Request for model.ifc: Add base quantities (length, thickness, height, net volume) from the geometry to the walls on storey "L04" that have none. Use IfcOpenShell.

First a look at what the model holds.

```python
import ifcopenshell
import ifcopenshell.util.element
import ifcopenshell.util.unit

model = ifcopenshell.open("model.ifc")
print(model.schema)
for unit_type in ("LENGTHUNIT", "AREAUNIT", "VOLUMEUNIT"):
    print(unit_type, ifcopenshell.util.unit.calculate_unit_scale(model, unit_type))
storey = next(s for s in model.by_type("IfcBuildingStorey") if s.Name == "L04")
walls = [e for e in ifcopenshell.util.element.get_decomposition(storey) if e.is_a("IfcWall")]
for e in sorted(walls, key=lambda e: e.id()):
    print(e.id(), e.is_a(), e.Name, list(ifcopenshell.util.element.get_psets(e, qtos_only=True)), sep=" | ")
```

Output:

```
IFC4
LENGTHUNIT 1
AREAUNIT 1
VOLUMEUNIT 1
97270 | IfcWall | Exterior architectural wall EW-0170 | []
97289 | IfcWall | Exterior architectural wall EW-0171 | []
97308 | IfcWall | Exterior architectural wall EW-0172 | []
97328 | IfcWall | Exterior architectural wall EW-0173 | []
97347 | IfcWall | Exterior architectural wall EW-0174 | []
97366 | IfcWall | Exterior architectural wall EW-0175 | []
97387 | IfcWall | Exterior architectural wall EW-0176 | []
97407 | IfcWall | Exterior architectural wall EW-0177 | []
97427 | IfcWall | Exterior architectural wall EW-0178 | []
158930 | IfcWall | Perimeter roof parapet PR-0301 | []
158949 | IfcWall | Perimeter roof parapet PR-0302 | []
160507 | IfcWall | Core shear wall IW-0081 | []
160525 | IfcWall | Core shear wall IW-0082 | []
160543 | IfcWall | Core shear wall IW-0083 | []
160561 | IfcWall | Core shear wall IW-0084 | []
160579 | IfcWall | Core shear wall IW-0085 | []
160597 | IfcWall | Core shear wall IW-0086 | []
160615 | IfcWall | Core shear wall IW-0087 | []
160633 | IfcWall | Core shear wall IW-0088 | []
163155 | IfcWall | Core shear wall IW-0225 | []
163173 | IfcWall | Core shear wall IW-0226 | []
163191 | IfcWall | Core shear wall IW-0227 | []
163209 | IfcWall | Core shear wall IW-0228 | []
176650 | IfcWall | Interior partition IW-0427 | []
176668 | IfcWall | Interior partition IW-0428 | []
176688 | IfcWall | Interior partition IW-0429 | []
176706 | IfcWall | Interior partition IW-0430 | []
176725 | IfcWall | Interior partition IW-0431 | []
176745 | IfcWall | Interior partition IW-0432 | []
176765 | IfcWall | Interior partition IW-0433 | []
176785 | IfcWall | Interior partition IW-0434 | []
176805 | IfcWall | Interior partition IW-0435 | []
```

```python
import ifcopenshell
import ifcopenshell.api.pset
import ifcopenshell.geom
import ifcopenshell.util.element
import ifcopenshell.util.shape
import ifcopenshell.util.unit

model = ifcopenshell.open("model.ifc")
unit_scale = ifcopenshell.util.unit.calculate_unit_scale(model)
volume_scale = ifcopenshell.util.unit.calculate_unit_scale(model, "VOLUMEUNIT")
settings = ifcopenshell.geom.settings()

storey = next(s for s in model.by_type("IfcBuildingStorey") if s.Name == "L04")
walls = [e for e in ifcopenshell.util.element.get_decomposition(storey) if e.is_a("IfcWall")]

for e in sorted(walls, key=lambda e: e.id()):
    if ifcopenshell.util.element.get_psets(e, qtos_only=True, should_inherit=False):
        continue
    # Geometry comes back in metres, in the element's own axes.
    shape = ifcopenshell.geom.create_shape(settings, e)
    values = {
        "Length": ifcopenshell.util.shape.get_x(shape.geometry) / unit_scale,
        "Width": ifcopenshell.util.shape.get_y(shape.geometry) / unit_scale,
        "Height": ifcopenshell.util.shape.get_z(shape.geometry) / unit_scale,
        "NetVolume": ifcopenshell.util.shape.get_volume(shape.geometry) / volume_scale,
    }
    qto = ifcopenshell.api.pset.add_qto(model, product=e, name="Qto_WallBaseQuantities")
    ifcopenshell.api.pset.edit_qto(model, qto=qto, properties=values)
    print(e.id(), {k: round(v, 3) for k, v in values.items()})

model.write("model_updated.ifc")
```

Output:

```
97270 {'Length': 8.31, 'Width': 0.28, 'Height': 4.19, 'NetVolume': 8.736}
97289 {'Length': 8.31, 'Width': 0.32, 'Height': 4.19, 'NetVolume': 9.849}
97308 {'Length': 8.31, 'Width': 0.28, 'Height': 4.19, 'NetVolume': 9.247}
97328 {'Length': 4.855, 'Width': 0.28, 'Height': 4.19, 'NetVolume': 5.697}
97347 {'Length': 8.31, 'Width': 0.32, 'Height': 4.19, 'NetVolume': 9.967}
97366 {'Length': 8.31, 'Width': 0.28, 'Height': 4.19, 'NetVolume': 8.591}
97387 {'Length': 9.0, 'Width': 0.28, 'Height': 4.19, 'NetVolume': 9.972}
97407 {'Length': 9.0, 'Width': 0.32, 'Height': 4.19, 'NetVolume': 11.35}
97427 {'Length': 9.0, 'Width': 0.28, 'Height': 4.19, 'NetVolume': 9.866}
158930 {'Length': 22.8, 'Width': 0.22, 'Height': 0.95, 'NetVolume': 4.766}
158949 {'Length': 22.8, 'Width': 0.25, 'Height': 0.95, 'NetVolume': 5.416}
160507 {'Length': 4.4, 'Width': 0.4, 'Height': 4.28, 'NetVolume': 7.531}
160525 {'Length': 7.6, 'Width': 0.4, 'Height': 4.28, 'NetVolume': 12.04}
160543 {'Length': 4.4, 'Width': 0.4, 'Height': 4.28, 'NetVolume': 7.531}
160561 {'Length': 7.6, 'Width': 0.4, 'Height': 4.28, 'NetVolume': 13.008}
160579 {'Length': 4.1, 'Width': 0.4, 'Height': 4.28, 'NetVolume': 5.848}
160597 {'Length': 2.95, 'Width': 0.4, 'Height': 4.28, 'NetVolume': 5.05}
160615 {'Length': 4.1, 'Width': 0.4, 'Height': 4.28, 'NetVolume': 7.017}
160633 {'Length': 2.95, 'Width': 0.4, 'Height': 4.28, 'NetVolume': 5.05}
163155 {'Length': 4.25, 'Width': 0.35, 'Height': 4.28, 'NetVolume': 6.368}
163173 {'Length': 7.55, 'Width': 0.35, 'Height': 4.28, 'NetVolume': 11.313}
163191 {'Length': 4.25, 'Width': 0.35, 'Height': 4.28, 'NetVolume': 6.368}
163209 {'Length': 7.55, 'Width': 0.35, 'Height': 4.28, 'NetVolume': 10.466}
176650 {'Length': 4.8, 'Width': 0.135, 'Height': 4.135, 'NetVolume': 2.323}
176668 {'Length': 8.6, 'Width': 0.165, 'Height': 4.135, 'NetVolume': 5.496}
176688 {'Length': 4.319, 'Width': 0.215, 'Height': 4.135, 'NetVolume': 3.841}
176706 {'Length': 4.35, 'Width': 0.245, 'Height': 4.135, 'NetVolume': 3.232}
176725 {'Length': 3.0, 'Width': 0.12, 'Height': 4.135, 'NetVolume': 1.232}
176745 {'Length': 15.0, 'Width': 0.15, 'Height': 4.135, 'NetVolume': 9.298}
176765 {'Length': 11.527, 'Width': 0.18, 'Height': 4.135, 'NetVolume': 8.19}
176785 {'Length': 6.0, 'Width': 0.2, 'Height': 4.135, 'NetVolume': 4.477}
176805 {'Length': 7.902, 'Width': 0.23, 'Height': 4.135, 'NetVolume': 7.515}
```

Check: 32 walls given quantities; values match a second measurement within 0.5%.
